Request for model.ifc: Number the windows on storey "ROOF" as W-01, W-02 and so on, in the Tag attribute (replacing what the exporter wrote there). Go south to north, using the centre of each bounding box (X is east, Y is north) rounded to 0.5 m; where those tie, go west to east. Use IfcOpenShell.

First a look at what the model holds.

```python
import ifcopenshell
import ifcopenshell.util.element
import ifcopenshell.util.placement

model = ifcopenshell.open("model.ifc")
print(model.schema)
storey = next(s for s in model.by_type("IfcBuildingStorey") if s.Name == "ROOF")
windows = [e for e in ifcopenshell.util.element.get_decomposition(storey) if e.is_a("IfcWindow")]
for e in sorted(windows, key=lambda e: e.id()):
    origin = ifcopenshell.util.placement.get_local_placement(e.ObjectPlacement)[:3, 3]
    print(e.id(), e.Tag, e.Name, origin.round(2) + 0.0, sep=" | ")
```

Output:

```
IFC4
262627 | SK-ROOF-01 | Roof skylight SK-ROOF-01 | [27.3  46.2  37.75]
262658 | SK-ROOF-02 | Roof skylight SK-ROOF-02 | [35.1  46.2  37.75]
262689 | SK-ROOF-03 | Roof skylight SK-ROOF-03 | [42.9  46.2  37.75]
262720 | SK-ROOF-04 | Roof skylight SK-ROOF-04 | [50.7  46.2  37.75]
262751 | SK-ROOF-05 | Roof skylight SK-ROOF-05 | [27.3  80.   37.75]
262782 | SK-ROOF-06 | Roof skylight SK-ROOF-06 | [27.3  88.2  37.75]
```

```python
import ifcopenshell
import ifcopenshell.geom
import ifcopenshell.util.element
import ifcopenshell.util.shape

model = ifcopenshell.open("model.ifc")
settings = ifcopenshell.geom.settings()
settings.set("use-world-coords", True)


def centre(element):
    shape = ifcopenshell.geom.create_shape(settings, element)
    return ifcopenshell.util.shape.get_bbox_centroid(shape.geometry)


storey = next(s for s in model.by_type("IfcBuildingStorey") if s.Name == "ROOF")
windows = [e for e in ifcopenshell.util.element.get_decomposition(storey) if e.is_a("IfcWindow")]

# Insertion points can sit at a corner or the storey origin, so sort by the geometry (in metres).
centres = {e: centre(e) for e in windows}
windows.sort(key=lambda e: (round(centres[e][1] / 0.5), centres[e][0]))

for i, e in enumerate(windows, start=1):
    number = f"W-{i:02d}"
    e.Tag = number
    print(e.id(), number)

model.write("model_rev.ifc")
```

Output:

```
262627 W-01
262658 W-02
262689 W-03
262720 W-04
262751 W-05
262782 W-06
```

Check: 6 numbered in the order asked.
